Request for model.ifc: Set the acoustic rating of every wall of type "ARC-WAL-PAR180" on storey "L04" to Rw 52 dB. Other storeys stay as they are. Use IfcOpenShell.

First a look at what the model holds.

```python
import ifcopenshell
import ifcopenshell.util.element

model = ifcopenshell.open("model.ifc")
print(model.schema)
storey = next(s for s in model.by_type("IfcBuildingStorey") if s.Name == "L04")
walls = [e for e in ifcopenshell.util.element.get_decomposition(storey) if e.is_a("IfcWall")]
seen = {}
for e in walls:
    element_type = ifcopenshell.util.element.get_type(e)
    key = (element_type.Name if element_type != e and element_type else None, ifcopenshell.util.element.get_pset(e, "Pset_WallCommon", "AcousticRating"))
    seen[key] = seen.get(key, 0) + 1
for (name, value), count in sorted(seen.items(), key=str):
    print(count, "x", name, "|", value)
```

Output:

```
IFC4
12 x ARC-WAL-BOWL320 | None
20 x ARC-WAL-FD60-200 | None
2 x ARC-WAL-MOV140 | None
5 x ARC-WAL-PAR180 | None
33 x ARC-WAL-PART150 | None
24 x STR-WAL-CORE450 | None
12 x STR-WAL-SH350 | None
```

```python
import ifcopenshell
import ifcopenshell.api.pset
import ifcopenshell.util.element

model = ifcopenshell.open("model.ifc")

storey = next(s for s in model.by_type("IfcBuildingStorey") if s.Name == "L04")
walls = [e for e in ifcopenshell.util.element.get_decomposition(storey) if e.is_a("IfcWall")]

count = 0
for e in walls:
    element_type = ifcopenshell.util.element.get_type(e)
    if element_type in (None, e) or element_type.Name != "ARC-WAL-PAR180":
        continue
    # add_pset returns the element's existing set when there is one.
    pset = ifcopenshell.api.pset.add_pset(model, product=e, name="Pset_WallCommon")
    ifcopenshell.api.pset.edit_pset(model, pset=pset, properties={"AcousticRating": "Rw 52 dB"})
    count += 1

print(count, "walls updated")

model.write("model_rev.ifc")
```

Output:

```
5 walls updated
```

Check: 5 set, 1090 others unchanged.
